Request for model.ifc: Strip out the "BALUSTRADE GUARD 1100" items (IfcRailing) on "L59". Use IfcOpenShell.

First a look at what the model holds.

```python
import ifcopenshell
import ifcopenshell.util.element

model = ifcopenshell.open("model.ifc")
print(model.schema)
storey = next(s for s in model.by_type("IfcBuildingStorey") if s.Name == "L59")
railings = [e for e in ifcopenshell.util.element.get_decomposition(storey) if e.is_a("IfcRailing")]
seen = {}
for e in railings:
    element_type = ifcopenshell.util.element.get_type(e)
    name = element_type.Name if element_type not in (None, e) else None
    seen[name] = seen.get(name, 0) + 1
for name, count in sorted(seen.items(), key=str):
    print(count, "x", name)
```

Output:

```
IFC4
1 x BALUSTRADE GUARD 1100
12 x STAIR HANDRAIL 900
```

```python
import ifcopenshell
import ifcopenshell.api.root
import ifcopenshell.util.element

model = ifcopenshell.open("model.ifc")

storey = next(s for s in model.by_type("IfcBuildingStorey") if s.Name == "L59")
railings = [e for e in ifcopenshell.util.element.get_decomposition(storey) if e.is_a("IfcRailing")]
targets = [e for e in railings if (t := ifcopenshell.util.element.get_type(e)) not in (None, e) and t.Name == "BALUSTRADE GUARD 1100"]

for e in targets:
    ifcopenshell.api.root.remove_product(model, product=e)
print(len(targets), "removed")

model.write("model_edited.ifc")
```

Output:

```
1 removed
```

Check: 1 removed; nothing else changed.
